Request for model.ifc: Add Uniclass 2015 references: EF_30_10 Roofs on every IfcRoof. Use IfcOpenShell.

First a look at what the model holds.

```python
import ifcopenshell

model = ifcopenshell.open("model.ifc")
print(model.schema)
print("classifications:", [c.Name for c in model.by_type("IfcClassification")])
for ifc_class in ("IfcDoor", "IfcRoof", "IfcStair", "IfcWall", "IfcWindow"):
    print(ifc_class, len(model.by_type(ifc_class)))
```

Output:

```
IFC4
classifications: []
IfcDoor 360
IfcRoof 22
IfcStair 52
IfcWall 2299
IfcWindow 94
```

```python
import ifcopenshell
import ifcopenshell.api.classification

model = ifcopenshell.open("model.ifc")

system = ifcopenshell.api.classification.add_classification(model, classification="Uniclass 2015")

codes = {
    "IfcRoof": ("EF_30_10", "Roofs"),
}
for ifc_class, (code, name) in codes.items():
    products = model.by_type(ifc_class)
    ifcopenshell.api.classification.add_reference(
        model, products=products, classification=system, identification=code, name=name
    )
    print(code, len(products))

model.write("model_v2.ifc")
```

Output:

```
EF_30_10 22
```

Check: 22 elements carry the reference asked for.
